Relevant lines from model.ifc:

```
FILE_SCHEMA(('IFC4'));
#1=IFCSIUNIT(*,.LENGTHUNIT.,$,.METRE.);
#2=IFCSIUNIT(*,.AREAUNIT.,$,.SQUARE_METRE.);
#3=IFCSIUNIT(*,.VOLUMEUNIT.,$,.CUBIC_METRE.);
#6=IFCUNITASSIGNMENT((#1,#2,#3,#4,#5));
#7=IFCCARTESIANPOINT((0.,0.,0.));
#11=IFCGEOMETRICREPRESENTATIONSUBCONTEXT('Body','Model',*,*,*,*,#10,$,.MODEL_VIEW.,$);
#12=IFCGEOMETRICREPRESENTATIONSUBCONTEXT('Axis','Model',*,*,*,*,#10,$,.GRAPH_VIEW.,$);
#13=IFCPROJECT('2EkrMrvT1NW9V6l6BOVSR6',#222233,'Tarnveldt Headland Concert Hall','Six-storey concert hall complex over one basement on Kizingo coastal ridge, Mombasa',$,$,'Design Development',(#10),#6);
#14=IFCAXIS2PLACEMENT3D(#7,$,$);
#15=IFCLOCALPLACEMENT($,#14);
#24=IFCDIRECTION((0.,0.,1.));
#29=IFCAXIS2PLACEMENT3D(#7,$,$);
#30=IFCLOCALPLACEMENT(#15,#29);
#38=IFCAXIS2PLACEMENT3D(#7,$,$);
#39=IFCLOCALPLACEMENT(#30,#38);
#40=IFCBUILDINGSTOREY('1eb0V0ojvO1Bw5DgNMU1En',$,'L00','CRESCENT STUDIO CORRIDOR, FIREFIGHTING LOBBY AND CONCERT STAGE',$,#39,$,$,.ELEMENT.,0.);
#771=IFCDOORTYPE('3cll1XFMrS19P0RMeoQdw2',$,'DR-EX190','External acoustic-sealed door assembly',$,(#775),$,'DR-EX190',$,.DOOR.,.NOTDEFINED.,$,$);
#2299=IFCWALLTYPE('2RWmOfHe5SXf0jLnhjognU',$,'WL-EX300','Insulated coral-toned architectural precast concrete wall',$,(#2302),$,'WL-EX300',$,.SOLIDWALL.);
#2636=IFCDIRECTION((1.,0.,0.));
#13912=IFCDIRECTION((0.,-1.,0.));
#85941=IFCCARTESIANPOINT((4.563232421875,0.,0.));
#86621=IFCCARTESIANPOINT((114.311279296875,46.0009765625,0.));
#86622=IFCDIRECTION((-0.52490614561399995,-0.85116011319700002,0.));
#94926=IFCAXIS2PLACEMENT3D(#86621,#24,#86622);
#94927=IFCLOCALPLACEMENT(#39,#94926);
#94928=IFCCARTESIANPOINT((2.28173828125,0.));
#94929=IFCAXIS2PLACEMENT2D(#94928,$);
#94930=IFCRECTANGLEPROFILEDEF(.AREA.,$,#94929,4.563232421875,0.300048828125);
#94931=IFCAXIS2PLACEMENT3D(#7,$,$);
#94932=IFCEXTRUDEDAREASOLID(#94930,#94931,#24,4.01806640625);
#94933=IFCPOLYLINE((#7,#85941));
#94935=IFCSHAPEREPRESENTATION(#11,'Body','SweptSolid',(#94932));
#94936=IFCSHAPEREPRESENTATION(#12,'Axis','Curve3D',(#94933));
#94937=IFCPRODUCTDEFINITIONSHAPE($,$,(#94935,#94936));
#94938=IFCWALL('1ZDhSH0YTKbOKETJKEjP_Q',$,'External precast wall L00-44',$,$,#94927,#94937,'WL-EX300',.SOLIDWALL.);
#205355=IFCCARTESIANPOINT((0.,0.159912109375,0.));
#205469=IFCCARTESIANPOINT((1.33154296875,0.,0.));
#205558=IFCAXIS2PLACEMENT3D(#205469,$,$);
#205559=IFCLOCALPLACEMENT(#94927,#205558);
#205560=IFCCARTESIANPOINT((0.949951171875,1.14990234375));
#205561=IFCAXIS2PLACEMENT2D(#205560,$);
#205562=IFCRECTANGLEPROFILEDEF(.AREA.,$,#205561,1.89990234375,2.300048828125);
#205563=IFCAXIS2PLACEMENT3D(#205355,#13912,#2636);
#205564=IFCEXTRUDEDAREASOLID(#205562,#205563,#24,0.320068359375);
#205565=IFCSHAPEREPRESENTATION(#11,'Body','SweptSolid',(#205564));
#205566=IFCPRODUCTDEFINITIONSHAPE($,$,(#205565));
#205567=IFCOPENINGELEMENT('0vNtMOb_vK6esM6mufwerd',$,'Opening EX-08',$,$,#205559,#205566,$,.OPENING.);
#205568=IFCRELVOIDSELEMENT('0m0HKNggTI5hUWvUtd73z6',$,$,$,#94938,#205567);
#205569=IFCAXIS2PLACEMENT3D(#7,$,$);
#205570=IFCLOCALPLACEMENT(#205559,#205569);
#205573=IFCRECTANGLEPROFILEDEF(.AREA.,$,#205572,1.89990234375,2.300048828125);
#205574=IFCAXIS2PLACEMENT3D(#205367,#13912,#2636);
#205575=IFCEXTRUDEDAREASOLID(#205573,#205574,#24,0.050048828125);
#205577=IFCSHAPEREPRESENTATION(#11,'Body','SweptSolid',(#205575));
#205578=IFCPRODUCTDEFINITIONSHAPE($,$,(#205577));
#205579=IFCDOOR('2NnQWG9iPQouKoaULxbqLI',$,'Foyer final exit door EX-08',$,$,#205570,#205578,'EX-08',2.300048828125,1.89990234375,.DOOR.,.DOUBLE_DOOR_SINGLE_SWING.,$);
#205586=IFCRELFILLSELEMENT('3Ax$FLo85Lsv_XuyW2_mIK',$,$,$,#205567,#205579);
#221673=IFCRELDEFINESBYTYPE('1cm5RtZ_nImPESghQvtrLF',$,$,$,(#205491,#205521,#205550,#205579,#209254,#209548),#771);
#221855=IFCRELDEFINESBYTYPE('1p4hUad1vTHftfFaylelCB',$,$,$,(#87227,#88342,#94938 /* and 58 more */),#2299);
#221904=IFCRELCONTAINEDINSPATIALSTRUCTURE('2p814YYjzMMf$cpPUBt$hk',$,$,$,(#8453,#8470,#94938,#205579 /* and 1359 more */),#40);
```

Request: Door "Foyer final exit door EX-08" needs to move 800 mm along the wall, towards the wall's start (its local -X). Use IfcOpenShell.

```python
import ifcopenshell
import ifcopenshell.api.geometry
import ifcopenshell.util.placement
import ifcopenshell.util.unit

model = ifcopenshell.open("model.ifc")
unit_scale = ifcopenshell.util.unit.calculate_unit_scale(model)

door = model.by_guid("2NnQWG9iPQouKoaULxbqLI")
opening = door.FillsVoids[0].RelatingOpeningElement
wall = opening.VoidsElements[0].RelatingBuildingElement

wall_matrix = ifcopenshell.util.placement.get_local_placement(wall.ObjectPlacement)
shift = wall_matrix[:3, 0] * -0.8 / unit_scale
before = ifcopenshell.util.placement.get_local_placement(door.ObjectPlacement)[:3, 3].copy()

# The door is placed relative to its opening, so it follows when the opening moves.
matrix = ifcopenshell.util.placement.get_local_placement(opening.ObjectPlacement)
matrix[:3, 3] += shift
ifcopenshell.api.geometry.edit_object_placement(
    model, product=opening, matrix=matrix, is_si=False, should_transform_children=True
)

after = ifcopenshell.util.placement.get_local_placement(door.ObjectPlacement)[:3, 3]
print("door moved by", (after - before).round(3) + 0.0)

model.write("model-out.ifc")
```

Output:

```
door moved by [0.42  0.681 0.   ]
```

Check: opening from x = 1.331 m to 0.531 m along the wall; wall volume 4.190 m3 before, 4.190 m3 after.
